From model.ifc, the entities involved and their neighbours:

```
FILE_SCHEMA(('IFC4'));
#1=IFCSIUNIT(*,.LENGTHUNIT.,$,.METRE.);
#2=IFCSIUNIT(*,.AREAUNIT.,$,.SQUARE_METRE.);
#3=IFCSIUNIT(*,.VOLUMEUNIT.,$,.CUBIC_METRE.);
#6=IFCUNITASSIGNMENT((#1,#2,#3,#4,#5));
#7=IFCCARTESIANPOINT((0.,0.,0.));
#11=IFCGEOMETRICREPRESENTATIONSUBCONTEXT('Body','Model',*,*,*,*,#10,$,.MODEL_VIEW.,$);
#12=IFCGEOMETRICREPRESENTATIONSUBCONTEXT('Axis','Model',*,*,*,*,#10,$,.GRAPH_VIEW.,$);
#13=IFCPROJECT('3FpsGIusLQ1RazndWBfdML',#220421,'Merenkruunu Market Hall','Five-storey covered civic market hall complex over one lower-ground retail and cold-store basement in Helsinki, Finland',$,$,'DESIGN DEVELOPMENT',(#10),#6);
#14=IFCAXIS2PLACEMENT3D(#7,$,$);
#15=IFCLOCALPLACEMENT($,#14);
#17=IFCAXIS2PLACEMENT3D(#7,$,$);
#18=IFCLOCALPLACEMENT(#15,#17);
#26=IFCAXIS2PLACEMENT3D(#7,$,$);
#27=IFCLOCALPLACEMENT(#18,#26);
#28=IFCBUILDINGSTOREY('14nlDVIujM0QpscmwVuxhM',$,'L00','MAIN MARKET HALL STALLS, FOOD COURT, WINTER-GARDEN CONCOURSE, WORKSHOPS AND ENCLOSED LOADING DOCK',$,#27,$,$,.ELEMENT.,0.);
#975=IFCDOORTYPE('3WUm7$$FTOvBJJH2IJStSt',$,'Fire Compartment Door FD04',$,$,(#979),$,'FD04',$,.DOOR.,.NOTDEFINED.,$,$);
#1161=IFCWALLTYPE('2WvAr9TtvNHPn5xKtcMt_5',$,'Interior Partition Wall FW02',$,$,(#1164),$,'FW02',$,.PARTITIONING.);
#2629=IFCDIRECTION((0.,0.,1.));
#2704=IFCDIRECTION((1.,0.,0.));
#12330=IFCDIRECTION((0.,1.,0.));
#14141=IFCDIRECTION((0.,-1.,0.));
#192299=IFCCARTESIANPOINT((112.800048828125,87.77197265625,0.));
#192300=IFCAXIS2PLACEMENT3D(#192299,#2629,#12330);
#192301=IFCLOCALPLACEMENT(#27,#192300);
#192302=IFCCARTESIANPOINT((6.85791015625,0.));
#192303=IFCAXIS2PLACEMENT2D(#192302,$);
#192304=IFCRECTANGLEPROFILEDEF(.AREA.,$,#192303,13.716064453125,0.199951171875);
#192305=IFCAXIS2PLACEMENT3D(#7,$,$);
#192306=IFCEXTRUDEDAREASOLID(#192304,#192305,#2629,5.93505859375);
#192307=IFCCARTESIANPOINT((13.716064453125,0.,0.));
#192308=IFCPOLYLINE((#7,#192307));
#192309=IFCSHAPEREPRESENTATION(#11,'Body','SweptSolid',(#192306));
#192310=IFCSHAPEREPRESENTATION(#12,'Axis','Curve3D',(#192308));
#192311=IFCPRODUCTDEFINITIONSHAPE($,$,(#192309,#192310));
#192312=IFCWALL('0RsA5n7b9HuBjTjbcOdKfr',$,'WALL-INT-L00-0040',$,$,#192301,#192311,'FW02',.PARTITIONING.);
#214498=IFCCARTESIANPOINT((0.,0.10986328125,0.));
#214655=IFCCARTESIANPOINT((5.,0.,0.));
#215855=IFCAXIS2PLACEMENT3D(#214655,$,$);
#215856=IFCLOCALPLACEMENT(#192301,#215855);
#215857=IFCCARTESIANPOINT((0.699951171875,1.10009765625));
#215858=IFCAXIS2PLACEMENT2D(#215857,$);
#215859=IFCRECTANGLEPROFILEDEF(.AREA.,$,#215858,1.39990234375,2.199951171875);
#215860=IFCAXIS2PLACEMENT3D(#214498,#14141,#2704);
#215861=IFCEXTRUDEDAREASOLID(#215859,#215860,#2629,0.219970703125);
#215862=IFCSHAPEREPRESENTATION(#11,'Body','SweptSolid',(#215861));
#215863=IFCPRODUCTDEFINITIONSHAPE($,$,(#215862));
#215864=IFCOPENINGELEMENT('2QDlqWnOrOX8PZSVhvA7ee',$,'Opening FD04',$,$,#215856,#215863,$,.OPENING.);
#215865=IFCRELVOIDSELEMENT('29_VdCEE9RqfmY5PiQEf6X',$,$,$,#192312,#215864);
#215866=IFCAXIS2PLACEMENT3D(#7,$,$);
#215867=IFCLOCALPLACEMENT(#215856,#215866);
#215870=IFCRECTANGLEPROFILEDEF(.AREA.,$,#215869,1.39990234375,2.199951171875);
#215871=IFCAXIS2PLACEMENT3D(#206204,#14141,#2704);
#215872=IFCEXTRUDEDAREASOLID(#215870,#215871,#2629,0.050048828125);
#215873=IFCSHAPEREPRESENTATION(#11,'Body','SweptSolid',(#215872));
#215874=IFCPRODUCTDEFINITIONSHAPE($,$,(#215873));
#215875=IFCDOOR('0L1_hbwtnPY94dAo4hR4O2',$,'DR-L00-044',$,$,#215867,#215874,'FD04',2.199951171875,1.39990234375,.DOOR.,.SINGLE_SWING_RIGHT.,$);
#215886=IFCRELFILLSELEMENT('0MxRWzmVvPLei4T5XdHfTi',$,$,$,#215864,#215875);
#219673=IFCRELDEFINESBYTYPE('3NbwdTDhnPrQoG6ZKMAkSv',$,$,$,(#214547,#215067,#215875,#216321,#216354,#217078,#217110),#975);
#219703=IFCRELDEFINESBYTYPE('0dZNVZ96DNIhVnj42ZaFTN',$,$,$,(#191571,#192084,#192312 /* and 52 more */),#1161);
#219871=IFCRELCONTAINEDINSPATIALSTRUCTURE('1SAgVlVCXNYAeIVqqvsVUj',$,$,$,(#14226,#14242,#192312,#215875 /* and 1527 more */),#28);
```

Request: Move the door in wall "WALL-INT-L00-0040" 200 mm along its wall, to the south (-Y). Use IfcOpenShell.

```python
import ifcopenshell
import ifcopenshell.api.geometry
import ifcopenshell.util.placement
import ifcopenshell.util.unit

model = ifcopenshell.open("model.ifc")
unit_scale = ifcopenshell.util.unit.calculate_unit_scale(model)

door = model.by_guid("0L1_hbwtnPY94dAo4hR4O2")
opening = door.FillsVoids[0].RelatingOpeningElement
wall = opening.VoidsElements[0].RelatingBuildingElement

wall_matrix = ifcopenshell.util.placement.get_local_placement(wall.ObjectPlacement)
shift = wall_matrix[:3, 0] * -0.2 / unit_scale
before = ifcopenshell.util.placement.get_local_placement(door.ObjectPlacement)[:3, 3].copy()

# The door is placed relative to its opening, so it follows when the opening moves.
matrix = ifcopenshell.util.placement.get_local_placement(opening.ObjectPlacement)
matrix[:3, 3] += shift
ifcopenshell.api.geometry.edit_object_placement(
    model, product=opening, matrix=matrix, is_si=False, should_transform_children=True
)

after = ifcopenshell.util.placement.get_local_placement(door.ObjectPlacement)[:3, 3]
print("door moved by", (after - before).round(3) + 0.0)

model.write("model_edited.ifc")
```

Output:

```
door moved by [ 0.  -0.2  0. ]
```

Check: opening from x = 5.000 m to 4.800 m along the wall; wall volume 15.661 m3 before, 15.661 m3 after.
